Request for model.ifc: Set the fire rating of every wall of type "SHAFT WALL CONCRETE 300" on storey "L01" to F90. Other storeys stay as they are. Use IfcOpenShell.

First a look at what the model holds.

```python
import ifcopenshell
import ifcopenshell.util.element

model = ifcopenshell.open("model.ifc")
print(model.schema)
storey = next(s for s in model.by_type("IfcBuildingStorey") if s.Name == "L01")
walls = [e for e in ifcopenshell.util.element.get_decomposition(storey) if e.is_a("IfcWall")]
seen = {}
for e in walls:
    element_type = ifcopenshell.util.element.get_type(e)
    key = (element_type.Name if element_type != e and element_type else None, ifcopenshell.util.element.get_pset(e, "Pset_WallCommon", "FireRating"))
    seen[key] = seen.get(key, 0) + 1
for (name, value), count in sorted(seen.items(), key=str):
    print(count, "x", name, "|", value)
```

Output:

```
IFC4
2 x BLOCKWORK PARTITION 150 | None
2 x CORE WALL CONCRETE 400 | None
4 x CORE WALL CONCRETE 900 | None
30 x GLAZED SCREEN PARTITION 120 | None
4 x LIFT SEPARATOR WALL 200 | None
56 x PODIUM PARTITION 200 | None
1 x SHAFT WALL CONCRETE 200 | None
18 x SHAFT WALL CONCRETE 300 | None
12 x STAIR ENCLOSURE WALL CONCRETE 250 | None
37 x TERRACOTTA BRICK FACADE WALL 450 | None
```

```python
import ifcopenshell
import ifcopenshell.api.pset
import ifcopenshell.util.element

model = ifcopenshell.open("model.ifc")

storey = next(s for s in model.by_type("IfcBuildingStorey") if s.Name == "L01")
walls = [e for e in ifcopenshell.util.element.get_decomposition(storey) if e.is_a("IfcWall")]

count = 0
for e in walls:
    element_type = ifcopenshell.util.element.get_type(e)
    if element_type in (None, e) or element_type.Name != "SHAFT WALL CONCRETE 300":
        continue
    found = ifcopenshell.util.element.get_pset(e, "Pset_WallCommon", should_inherit=False)
    if found:
        pset = model.by_id(found["id"])
        if len(ifcopenshell.util.element.get_elements_by_pset(pset)) > 1:
            pset = ifcopenshell.api.pset.unshare_pset(model, products=[e], pset=pset)[0]
    else:
        pset = ifcopenshell.api.pset.add_pset(model, product=e, name="Pset_WallCommon")
    ifcopenshell.api.pset.edit_pset(model, pset=pset, properties={"FireRating": "F90"})
    count += 1

print(count, "walls updated")

model.write("model_updated.ifc")
```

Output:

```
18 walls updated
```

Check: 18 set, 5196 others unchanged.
